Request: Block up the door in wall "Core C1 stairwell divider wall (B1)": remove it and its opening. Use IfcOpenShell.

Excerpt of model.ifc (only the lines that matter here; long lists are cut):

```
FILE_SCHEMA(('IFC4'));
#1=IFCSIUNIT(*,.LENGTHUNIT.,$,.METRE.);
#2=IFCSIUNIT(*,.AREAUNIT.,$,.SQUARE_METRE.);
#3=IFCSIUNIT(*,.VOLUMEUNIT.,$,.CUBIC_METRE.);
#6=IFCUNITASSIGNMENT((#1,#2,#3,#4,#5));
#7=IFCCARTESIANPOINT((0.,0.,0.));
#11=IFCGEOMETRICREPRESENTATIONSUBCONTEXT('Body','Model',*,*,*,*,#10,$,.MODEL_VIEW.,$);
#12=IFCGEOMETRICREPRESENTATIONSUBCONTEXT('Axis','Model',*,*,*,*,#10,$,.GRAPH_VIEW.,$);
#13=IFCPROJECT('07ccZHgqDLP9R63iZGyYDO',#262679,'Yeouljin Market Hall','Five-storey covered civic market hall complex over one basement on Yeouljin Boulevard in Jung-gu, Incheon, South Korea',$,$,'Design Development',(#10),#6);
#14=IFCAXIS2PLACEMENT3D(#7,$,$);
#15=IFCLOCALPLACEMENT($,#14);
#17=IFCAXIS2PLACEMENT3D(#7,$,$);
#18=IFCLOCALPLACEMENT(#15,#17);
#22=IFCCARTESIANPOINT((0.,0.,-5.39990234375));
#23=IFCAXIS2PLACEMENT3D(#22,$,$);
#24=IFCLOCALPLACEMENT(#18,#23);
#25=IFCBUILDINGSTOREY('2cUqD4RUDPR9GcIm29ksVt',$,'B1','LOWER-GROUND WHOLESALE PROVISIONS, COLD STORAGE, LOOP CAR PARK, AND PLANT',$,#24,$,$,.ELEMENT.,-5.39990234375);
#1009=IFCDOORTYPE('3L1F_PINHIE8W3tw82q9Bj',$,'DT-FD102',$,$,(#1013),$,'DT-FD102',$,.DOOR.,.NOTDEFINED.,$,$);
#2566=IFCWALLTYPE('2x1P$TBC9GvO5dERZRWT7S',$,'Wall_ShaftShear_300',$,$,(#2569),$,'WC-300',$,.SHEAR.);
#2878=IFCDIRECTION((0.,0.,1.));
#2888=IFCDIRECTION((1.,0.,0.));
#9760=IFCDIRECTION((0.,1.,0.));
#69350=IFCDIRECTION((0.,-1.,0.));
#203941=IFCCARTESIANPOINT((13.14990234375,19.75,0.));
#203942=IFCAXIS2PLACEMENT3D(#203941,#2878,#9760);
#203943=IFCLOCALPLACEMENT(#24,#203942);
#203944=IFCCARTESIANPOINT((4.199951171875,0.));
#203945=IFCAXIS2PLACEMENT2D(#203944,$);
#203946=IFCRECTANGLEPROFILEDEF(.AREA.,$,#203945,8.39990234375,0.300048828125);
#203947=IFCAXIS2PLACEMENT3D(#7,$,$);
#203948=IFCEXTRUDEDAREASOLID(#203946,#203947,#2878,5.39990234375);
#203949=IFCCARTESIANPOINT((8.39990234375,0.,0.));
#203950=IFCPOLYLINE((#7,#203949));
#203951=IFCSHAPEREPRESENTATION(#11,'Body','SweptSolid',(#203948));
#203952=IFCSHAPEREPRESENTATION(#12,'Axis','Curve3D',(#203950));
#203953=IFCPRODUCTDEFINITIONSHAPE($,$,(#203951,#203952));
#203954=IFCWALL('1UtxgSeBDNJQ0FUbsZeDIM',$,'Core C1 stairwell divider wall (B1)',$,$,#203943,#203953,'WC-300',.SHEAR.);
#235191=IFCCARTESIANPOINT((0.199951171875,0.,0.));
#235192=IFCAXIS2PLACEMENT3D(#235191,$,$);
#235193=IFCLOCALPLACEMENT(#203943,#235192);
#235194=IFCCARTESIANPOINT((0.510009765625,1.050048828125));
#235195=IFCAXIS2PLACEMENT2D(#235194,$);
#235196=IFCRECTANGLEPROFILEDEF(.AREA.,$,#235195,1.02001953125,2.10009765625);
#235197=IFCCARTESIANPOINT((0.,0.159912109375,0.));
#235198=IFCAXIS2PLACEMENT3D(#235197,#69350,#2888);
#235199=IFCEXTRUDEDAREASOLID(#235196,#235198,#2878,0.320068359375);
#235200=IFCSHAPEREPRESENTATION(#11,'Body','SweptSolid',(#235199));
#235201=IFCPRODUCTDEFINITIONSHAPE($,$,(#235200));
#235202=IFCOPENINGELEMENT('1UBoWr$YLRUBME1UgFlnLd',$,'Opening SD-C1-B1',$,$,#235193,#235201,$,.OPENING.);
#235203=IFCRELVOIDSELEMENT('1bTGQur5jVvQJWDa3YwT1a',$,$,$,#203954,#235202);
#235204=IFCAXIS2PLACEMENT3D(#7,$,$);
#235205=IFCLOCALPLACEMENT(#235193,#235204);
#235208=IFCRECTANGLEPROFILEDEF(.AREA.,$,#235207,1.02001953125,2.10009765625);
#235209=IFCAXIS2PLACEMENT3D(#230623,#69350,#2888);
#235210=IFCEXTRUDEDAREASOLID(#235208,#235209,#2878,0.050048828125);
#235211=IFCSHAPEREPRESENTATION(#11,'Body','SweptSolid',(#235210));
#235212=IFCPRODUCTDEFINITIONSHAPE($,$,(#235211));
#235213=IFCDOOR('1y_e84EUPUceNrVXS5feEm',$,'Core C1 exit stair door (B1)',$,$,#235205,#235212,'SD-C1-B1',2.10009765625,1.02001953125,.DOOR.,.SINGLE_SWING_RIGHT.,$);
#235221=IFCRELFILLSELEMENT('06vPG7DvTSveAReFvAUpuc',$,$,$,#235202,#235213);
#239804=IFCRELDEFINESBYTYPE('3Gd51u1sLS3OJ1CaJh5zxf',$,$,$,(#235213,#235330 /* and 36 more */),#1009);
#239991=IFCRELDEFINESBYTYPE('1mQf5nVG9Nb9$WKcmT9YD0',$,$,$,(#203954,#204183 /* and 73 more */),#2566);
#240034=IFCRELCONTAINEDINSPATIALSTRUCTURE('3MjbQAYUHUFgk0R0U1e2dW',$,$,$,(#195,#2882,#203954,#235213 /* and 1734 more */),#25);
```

```python
import ifcopenshell
import ifcopenshell.api.feature
import ifcopenshell.api.root
import ifcopenshell.geom
import ifcopenshell.util.shape

model = ifcopenshell.open("model.ifc")
settings = ifcopenshell.geom.settings()


def volume(element):
    """Net volume in cubic metres, openings subtracted."""
    shape = ifcopenshell.geom.create_shape(settings, element)
    return ifcopenshell.util.shape.get_volume(shape.geometry)


door = model.by_guid("1y_e84EUPUceNrVXS5feEm")
opening = door.FillsVoids[0].RelatingOpeningElement
wall = opening.VoidsElements[0].RelatingBuildingElement
before = volume(wall)

ifcopenshell.api.root.remove_product(model, product=door)
ifcopenshell.api.feature.remove_feature(model, feature=opening)

after = volume(wall)

print(f"wall volume {before:.3f} -> {after:.3f} m3")

model.write("model_rev.ifc")
```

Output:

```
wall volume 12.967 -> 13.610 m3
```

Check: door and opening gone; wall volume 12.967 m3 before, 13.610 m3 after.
